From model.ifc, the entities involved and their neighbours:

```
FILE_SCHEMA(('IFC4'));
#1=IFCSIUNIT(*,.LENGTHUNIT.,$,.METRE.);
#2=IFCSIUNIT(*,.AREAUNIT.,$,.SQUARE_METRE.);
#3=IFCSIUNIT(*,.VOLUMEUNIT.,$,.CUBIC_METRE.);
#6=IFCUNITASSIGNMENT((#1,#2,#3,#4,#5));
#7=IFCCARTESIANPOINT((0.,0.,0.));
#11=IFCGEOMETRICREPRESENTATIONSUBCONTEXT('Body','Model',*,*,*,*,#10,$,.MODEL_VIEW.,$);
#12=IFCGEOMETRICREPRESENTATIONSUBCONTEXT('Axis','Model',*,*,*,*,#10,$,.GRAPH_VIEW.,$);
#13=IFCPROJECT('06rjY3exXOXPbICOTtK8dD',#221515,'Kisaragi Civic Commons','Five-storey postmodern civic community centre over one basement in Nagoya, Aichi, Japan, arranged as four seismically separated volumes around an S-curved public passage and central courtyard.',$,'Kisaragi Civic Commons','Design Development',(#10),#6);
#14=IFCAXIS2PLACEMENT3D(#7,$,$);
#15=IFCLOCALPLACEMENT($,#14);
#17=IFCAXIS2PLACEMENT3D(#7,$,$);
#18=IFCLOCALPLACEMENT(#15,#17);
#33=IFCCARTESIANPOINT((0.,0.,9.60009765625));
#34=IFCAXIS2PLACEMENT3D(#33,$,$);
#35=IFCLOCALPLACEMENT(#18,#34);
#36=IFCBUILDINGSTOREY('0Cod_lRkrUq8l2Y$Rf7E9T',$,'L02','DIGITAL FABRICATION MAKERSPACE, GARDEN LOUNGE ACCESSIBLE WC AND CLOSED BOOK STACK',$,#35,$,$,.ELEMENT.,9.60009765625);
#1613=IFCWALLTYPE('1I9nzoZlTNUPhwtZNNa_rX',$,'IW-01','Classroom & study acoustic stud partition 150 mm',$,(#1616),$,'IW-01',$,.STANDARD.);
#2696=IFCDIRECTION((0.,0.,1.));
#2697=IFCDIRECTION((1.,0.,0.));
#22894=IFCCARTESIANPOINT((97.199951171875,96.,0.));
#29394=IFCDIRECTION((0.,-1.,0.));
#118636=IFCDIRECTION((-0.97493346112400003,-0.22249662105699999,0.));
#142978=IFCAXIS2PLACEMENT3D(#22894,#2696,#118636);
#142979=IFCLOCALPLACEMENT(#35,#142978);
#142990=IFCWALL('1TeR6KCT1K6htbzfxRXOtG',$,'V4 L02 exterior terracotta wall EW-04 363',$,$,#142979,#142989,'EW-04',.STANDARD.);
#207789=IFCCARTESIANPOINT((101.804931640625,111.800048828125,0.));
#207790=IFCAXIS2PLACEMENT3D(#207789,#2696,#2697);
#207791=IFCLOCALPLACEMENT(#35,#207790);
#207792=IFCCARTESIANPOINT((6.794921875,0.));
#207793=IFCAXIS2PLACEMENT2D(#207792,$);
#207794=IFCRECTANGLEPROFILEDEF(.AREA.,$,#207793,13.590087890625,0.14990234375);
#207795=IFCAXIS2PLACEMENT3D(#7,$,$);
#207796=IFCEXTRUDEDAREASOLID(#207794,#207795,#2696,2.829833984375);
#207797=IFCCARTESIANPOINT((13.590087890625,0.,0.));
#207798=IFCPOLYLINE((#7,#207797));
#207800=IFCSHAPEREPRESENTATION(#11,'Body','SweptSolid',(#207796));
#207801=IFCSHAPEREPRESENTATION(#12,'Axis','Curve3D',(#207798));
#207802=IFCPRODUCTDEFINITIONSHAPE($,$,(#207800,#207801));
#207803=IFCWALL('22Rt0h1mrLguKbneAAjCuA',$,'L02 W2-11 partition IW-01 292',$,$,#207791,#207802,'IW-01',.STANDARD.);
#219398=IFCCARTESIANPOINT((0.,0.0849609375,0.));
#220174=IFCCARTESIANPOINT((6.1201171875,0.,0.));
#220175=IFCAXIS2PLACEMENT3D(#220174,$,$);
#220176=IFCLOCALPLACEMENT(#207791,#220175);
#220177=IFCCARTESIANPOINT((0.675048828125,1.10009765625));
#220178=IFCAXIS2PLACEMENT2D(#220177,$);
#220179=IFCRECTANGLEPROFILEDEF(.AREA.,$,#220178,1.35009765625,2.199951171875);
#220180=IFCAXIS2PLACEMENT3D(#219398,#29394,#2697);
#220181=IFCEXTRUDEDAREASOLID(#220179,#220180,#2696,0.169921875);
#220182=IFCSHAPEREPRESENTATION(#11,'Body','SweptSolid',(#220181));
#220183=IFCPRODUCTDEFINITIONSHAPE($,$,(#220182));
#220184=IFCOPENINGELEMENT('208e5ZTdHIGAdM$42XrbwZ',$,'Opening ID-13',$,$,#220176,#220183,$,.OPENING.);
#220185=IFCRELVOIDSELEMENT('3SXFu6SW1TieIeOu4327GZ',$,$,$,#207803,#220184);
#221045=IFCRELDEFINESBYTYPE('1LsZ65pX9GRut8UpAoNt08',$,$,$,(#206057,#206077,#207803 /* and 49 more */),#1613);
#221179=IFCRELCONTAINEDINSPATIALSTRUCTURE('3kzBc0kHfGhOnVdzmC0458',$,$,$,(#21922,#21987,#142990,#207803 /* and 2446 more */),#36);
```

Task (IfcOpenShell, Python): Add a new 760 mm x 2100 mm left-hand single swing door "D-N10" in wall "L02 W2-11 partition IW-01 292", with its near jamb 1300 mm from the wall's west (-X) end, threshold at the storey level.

```python
import numpy as np
import ifcopenshell
import ifcopenshell.api.feature
import ifcopenshell.api.geometry
import ifcopenshell.api.root
import ifcopenshell.api.spatial
import ifcopenshell.geom
import ifcopenshell.util.element
import ifcopenshell.util.placement
import ifcopenshell.util.representation
import ifcopenshell.util.shape
import ifcopenshell.util.unit

model = ifcopenshell.open("model.ifc")
unit_scale = ifcopenshell.util.unit.calculate_unit_scale(model)
settings = ifcopenshell.geom.settings()


def volume(element):
    """Net volume in cubic metres, openings subtracted."""
    shape = ifcopenshell.geom.create_shape(settings, element)
    return ifcopenshell.util.shape.get_volume(shape.geometry)


wall = model.by_id(207803)
storey = ifcopenshell.util.element.get_container(wall, ifc_class="IfcBuildingStorey")
context = ifcopenshell.util.representation.get_context(model, "Model", "Body", "MODEL_VIEW")
before = volume(wall)

width, height, from_end, sill = 0.76, 2.1, 1.3, 0.0  # metres

# The wall runs along its own X axis, and the end named is its -X end.
wall_shape = ifcopenshell.geom.create_shape(settings, wall)
x, y, z = ifcopenshell.util.shape.get_vertices(wall_shape.geometry).T
start = x.min() + from_end
face, thickness = float(y.min()), float(y.max() - y.min())
wall_matrix = ifcopenshell.util.placement.get_local_placement(wall.ObjectPlacement)
level = ifcopenshell.util.placement.get_local_placement(storey.ObjectPlacement)[2, 3]


def in_wall(x, y):
    """Placement at x, y metres in the wall's axes, at sill height."""
    matrix = wall_matrix.copy()
    matrix[:, 3] = wall_matrix @ np.array([x / unit_scale, y / unit_scale, 0.0, 1.0])
    matrix[2, 3] = level + sill / unit_scale
    return matrix


# Opening: a box that overshoots both wall faces by 50 mm.
opening = ifcopenshell.api.root.create_entity(model, ifc_class="IfcOpeningElement", predefined_type="OPENING")
box = ifcopenshell.api.geometry.add_wall_representation(
    model, context=context, length=width, height=height, thickness=thickness + 0.1
)
ifcopenshell.api.geometry.assign_representation(model, product=opening, representation=box)
ifcopenshell.api.geometry.edit_object_placement(model, product=opening, matrix=in_wall(start, face - 0.05), is_si=False)
ifcopenshell.api.feature.add_feature(model, feature=opening, element=wall)

door = ifcopenshell.api.root.create_entity(model, ifc_class="IfcDoor", name="D-N10", predefined_type="DOOR")
door.OverallWidth, door.OverallHeight = width / unit_scale, height / unit_scale
door.OperationType = "SINGLE_SWING_LEFT"
body = ifcopenshell.api.geometry.add_door_representation(
    model,
    context=context,
    overall_width=door.OverallWidth,
    overall_height=door.OverallHeight,
    operation_type="SINGLE_SWING_LEFT",
    lining_properties={"LiningDepth": thickness / unit_scale, "ThresholdDepth": thickness / unit_scale},
)
ifcopenshell.api.geometry.assign_representation(model, product=door, representation=body)
ifcopenshell.api.spatial.assign_container(model, products=[door], relating_structure=storey)
ifcopenshell.api.feature.add_filling(model, opening=opening, element=door)

# The lining spans the wall, so the door starts at the wall face.
ifcopenshell.api.geometry.edit_object_placement(model, product=door, matrix=in_wall(start, face), is_si=False)

after = volume(wall)

print(f"wall volume {before:.3f} -> {after:.3f} m3")

model.write("model_updated.ifc")
```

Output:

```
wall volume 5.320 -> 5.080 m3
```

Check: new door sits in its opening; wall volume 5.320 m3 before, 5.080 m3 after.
